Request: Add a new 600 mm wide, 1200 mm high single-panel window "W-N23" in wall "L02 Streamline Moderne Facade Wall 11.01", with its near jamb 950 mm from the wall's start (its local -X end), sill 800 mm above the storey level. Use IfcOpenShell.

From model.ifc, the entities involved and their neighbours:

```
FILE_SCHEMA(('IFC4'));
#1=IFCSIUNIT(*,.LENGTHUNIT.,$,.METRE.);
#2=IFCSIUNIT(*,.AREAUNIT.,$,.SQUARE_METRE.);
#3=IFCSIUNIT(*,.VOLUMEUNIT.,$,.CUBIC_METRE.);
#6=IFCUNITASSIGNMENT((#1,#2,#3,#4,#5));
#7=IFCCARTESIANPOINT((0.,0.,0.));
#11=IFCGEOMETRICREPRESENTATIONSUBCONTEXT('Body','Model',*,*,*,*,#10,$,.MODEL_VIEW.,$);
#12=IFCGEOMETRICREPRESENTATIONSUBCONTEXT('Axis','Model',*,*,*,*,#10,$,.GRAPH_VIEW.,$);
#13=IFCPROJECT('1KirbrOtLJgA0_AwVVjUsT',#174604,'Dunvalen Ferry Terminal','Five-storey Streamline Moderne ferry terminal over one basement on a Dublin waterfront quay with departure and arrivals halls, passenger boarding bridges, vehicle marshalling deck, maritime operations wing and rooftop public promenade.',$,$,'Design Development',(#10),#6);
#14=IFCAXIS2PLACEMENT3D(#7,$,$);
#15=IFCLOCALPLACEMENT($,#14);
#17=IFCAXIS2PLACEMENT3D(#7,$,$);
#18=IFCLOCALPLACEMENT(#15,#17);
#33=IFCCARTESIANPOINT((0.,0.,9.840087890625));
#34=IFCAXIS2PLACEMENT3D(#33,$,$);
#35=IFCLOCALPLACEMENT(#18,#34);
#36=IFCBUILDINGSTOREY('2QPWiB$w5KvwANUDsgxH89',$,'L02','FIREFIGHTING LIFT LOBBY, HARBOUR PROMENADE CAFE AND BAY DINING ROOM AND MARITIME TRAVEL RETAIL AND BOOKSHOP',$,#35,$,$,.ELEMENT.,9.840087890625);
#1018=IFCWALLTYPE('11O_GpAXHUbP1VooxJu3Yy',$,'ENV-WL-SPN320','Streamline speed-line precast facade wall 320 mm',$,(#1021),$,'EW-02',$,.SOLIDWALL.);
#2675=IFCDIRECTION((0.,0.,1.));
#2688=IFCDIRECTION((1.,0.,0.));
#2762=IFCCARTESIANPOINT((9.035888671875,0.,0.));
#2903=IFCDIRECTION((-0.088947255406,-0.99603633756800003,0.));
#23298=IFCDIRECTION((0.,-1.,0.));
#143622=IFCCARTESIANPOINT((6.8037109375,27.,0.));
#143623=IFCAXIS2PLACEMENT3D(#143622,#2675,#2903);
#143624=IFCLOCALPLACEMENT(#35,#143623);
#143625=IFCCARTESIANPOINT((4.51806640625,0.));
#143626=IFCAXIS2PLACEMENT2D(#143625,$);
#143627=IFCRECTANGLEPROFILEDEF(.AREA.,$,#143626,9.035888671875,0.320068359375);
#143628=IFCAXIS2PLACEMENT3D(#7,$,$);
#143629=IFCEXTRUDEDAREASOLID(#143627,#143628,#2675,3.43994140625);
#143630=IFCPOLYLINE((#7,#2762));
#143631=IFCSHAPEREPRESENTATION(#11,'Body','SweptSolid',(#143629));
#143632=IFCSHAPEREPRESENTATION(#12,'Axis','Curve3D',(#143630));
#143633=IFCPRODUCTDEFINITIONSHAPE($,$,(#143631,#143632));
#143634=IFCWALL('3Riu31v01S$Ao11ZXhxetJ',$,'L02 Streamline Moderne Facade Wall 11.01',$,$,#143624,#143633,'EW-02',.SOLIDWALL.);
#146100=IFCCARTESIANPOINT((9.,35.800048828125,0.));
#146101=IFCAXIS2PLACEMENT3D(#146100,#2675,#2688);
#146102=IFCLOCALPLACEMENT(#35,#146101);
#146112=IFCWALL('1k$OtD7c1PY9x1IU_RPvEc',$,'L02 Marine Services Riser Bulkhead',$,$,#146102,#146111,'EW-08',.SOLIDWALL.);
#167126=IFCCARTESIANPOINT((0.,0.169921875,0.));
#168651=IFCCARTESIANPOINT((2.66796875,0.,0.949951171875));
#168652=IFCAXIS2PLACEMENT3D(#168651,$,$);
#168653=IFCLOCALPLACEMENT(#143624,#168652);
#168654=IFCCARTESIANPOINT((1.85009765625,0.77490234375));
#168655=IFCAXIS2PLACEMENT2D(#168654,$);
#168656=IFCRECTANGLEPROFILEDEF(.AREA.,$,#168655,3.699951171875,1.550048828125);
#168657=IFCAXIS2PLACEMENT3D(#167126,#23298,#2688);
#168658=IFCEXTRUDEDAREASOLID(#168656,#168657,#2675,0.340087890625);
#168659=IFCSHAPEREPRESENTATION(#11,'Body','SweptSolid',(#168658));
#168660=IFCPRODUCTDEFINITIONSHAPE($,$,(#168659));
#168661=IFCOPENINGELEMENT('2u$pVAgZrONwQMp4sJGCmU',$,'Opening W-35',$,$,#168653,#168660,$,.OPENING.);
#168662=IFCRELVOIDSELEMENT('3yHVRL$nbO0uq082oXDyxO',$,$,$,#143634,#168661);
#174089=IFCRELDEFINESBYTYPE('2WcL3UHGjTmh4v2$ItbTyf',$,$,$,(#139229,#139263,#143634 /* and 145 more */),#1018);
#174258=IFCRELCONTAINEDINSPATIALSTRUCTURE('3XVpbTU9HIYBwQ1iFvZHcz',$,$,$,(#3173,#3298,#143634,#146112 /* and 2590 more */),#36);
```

```python
import numpy as np
import ifcopenshell
import ifcopenshell.api.feature
import ifcopenshell.api.geometry
import ifcopenshell.api.root
import ifcopenshell.api.spatial
import ifcopenshell.geom
import ifcopenshell.util.element
import ifcopenshell.util.placement
import ifcopenshell.util.representation
import ifcopenshell.util.shape
import ifcopenshell.util.unit

model = ifcopenshell.open("model.ifc")
unit_scale = ifcopenshell.util.unit.calculate_unit_scale(model)
settings = ifcopenshell.geom.settings()


def volume(element):
    """Net volume in cubic metres, openings subtracted."""
    shape = ifcopenshell.geom.create_shape(settings, element)
    return ifcopenshell.util.shape.get_volume(shape.geometry)


wall = model.by_guid("3Riu31v01S$Ao11ZXhxetJ")
storey = ifcopenshell.util.element.get_container(wall, ifc_class="IfcBuildingStorey")
context = ifcopenshell.util.representation.get_context(model, "Model", "Body", "MODEL_VIEW")
before = volume(wall)

width, height, from_end, sill = 0.6, 1.2, 0.95, 0.8  # metres

# The wall runs along its own X axis, and the end named is its -X end.
wall_shape = ifcopenshell.geom.create_shape(settings, wall)
x, y, z = ifcopenshell.util.shape.get_vertices(wall_shape.geometry).T
start = x.min() + from_end
face, thickness = float(y.min()), float(y.max() - y.min())
wall_matrix = ifcopenshell.util.placement.get_local_placement(wall.ObjectPlacement)
level = ifcopenshell.util.placement.get_local_placement(storey.ObjectPlacement)[2, 3]


def in_wall(x, y):
    """Placement at x, y metres in the wall's axes, at sill height."""
    matrix = wall_matrix.copy()
    matrix[:, 3] = wall_matrix @ np.array([x / unit_scale, y / unit_scale, 0.0, 1.0])
    matrix[2, 3] = level + sill / unit_scale
    return matrix


# Opening: a box that overshoots both wall faces by 50 mm.
opening = ifcopenshell.api.root.create_entity(model, ifc_class="IfcOpeningElement", predefined_type="OPENING")
box = ifcopenshell.api.geometry.add_wall_representation(
    model, context=context, length=width, height=height, thickness=thickness + 0.1
)
ifcopenshell.api.geometry.assign_representation(model, product=opening, representation=box)
ifcopenshell.api.geometry.edit_object_placement(model, product=opening, matrix=in_wall(start, face - 0.05), is_si=False)
ifcopenshell.api.feature.add_feature(model, feature=opening, element=wall)

window = ifcopenshell.api.root.create_entity(model, ifc_class="IfcWindow", name="W-N23", predefined_type="WINDOW")
window.OverallWidth, window.OverallHeight = width / unit_scale, height / unit_scale
window.PartitioningType = "SINGLE_PANEL"
body = ifcopenshell.api.geometry.add_window_representation(
    model,
    context=context,
    overall_width=window.OverallWidth,
    overall_height=window.OverallHeight,
    partition_type="SINGLE_PANEL",
)
ifcopenshell.api.geometry.assign_representation(model, product=window, representation=body)
ifcopenshell.api.spatial.assign_container(model, products=[window], relating_structure=storey)
ifcopenshell.api.feature.add_filling(model, opening=opening, element=window)

# Centre the window in the wall's thickness.
ifcopenshell.api.geometry.edit_object_placement(model, product=window, matrix=in_wall(start, face), is_si=False)
window_shape = ifcopenshell.geom.create_shape(settings, window)
depth = ifcopenshell.util.shape.get_vertices(window_shape.geometry)[:, 1]
offset = face + thickness / 2 - (depth.min() + depth.max()) / 2
ifcopenshell.api.geometry.edit_object_placement(model, product=window, matrix=in_wall(start, offset), is_si=False)

after = volume(wall)

print(f"wall volume {before:.3f} -> {after:.3f} m3")

model.write("model_updated.ifc")
```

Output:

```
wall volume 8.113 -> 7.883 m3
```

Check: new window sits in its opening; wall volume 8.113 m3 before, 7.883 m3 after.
